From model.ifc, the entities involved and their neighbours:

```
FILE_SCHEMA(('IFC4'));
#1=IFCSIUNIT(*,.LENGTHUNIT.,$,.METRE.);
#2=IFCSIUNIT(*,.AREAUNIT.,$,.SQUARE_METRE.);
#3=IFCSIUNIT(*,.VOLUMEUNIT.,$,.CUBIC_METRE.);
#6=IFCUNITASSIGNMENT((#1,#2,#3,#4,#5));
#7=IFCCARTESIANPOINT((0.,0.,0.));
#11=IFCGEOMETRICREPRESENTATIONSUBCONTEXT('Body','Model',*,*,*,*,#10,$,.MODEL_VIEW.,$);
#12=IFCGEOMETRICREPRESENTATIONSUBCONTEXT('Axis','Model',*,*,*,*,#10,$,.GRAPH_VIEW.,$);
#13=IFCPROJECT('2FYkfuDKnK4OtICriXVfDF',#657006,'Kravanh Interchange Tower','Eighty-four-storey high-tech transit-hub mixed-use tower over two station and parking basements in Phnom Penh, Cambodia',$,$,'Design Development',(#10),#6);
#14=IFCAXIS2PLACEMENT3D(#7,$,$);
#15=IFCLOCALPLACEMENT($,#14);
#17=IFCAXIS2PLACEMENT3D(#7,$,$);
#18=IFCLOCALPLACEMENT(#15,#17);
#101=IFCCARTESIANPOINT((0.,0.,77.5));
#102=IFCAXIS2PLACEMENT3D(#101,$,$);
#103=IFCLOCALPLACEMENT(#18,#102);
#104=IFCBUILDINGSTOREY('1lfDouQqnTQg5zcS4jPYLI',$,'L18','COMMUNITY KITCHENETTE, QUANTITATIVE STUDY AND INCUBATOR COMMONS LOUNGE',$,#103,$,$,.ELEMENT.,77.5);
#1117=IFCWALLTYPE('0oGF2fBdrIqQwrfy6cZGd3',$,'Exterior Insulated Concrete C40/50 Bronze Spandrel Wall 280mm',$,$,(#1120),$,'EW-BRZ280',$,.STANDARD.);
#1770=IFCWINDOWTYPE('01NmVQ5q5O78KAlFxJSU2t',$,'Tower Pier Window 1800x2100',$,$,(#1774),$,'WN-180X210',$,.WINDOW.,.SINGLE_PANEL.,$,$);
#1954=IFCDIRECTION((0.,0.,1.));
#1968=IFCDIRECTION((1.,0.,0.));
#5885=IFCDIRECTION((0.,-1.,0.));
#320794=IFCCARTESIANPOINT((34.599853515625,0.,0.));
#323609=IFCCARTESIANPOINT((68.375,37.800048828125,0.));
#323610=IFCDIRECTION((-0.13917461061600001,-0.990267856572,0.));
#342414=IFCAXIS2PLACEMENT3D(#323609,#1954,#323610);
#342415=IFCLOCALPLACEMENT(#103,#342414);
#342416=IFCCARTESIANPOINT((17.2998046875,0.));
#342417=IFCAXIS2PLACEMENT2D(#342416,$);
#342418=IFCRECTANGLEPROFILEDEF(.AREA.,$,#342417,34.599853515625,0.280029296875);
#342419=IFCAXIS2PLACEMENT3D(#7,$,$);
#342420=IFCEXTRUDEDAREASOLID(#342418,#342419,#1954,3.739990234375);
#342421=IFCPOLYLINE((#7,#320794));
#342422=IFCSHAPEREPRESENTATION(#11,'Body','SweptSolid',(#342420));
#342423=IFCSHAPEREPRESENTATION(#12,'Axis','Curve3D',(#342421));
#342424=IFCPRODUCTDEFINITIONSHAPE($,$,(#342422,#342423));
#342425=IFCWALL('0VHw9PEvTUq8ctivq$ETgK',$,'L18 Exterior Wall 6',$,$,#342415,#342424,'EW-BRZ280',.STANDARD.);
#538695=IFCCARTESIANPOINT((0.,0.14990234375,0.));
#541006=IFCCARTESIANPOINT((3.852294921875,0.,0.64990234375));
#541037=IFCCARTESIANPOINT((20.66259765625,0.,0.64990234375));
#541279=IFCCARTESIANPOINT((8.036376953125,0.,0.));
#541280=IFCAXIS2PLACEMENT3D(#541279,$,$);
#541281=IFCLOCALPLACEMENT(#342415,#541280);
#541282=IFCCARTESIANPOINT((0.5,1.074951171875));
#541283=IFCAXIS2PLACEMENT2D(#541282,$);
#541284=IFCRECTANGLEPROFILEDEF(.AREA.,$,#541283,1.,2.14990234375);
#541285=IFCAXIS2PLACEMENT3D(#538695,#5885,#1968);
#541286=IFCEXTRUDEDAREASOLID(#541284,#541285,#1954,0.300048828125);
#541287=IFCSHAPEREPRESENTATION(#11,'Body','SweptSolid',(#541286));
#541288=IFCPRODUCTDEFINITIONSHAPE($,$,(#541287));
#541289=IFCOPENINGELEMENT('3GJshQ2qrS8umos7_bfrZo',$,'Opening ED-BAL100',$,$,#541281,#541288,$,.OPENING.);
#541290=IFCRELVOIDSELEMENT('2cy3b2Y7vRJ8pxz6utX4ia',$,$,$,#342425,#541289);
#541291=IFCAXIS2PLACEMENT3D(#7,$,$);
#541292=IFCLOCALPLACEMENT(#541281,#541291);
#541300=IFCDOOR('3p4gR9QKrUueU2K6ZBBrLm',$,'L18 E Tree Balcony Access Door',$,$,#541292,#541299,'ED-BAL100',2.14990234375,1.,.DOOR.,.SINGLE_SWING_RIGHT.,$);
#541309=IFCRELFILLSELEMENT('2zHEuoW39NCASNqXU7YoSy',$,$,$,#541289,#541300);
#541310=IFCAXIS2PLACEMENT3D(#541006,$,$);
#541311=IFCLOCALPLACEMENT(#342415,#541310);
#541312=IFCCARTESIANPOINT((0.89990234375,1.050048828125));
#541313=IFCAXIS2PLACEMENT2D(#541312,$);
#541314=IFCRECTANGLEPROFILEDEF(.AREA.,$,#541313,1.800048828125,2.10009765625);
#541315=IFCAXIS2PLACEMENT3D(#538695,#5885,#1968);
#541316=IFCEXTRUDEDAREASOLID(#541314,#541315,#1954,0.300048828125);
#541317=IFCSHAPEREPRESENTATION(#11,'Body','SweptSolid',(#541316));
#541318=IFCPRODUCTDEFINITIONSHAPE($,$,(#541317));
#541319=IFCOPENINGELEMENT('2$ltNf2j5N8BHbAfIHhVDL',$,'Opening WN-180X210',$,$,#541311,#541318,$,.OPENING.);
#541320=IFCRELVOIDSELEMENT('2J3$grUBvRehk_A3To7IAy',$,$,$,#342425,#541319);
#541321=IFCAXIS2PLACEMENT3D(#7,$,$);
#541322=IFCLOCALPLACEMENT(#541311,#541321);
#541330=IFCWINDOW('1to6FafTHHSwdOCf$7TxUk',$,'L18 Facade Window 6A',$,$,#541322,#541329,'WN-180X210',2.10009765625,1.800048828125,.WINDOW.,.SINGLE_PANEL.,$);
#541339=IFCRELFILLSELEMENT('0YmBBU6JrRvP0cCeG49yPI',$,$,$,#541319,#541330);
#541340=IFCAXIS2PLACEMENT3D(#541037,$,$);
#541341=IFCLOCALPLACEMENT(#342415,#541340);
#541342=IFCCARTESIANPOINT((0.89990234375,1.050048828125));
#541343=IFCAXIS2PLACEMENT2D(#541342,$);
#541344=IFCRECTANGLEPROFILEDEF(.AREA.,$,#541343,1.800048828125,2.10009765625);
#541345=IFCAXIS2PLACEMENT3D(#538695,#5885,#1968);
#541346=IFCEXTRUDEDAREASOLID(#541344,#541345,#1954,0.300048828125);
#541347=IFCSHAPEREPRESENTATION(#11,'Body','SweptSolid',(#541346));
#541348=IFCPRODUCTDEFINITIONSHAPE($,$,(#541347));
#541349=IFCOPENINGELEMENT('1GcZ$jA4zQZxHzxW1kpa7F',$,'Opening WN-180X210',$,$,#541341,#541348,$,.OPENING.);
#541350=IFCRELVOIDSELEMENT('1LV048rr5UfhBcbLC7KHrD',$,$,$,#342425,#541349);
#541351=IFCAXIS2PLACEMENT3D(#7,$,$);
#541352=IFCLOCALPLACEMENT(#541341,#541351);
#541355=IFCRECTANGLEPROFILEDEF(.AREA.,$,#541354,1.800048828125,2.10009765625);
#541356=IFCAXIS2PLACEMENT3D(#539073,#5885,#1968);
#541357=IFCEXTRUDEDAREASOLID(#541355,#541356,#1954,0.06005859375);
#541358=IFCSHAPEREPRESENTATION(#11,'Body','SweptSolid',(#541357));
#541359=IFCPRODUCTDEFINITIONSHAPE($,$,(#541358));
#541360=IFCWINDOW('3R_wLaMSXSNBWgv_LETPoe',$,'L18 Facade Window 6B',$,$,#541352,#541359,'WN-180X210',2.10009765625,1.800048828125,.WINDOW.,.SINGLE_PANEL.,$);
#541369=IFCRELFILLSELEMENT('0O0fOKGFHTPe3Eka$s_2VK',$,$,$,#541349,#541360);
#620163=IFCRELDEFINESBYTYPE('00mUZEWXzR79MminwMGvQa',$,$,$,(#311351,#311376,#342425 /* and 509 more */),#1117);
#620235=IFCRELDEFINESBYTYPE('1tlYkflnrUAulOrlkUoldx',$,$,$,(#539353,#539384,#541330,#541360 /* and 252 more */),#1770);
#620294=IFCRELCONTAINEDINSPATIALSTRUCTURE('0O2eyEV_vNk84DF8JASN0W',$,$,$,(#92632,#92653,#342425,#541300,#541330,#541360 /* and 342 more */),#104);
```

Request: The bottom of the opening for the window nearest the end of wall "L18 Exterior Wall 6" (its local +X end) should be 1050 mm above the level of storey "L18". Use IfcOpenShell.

```python
import numpy as np
import ifcopenshell
import ifcopenshell.api.geometry
import ifcopenshell.geom
import ifcopenshell.util.element
import ifcopenshell.util.placement
import ifcopenshell.util.shape
import ifcopenshell.util.unit

model = ifcopenshell.open("model.ifc")
unit_scale = ifcopenshell.util.unit.calculate_unit_scale(model)

window = model.by_guid("3R_wLaMSXSNBWgv_LETPoe")
opening = window.FillsVoids[0].RelatingOpeningElement
storey = ifcopenshell.util.element.get_container(window, ifc_class="IfcBuildingStorey")
level = ifcopenshell.util.placement.get_local_placement(storey.ObjectPlacement)[2, 3]

# The opening's origin need not be at the sill, so measure its lowest point.
shape = ifcopenshell.geom.create_shape(ifcopenshell.geom.settings(), opening)
bottom = ifcopenshell.util.shape.get_shape_bottom_elevation(shape, shape.geometry) / unit_scale
dz = level + 1.05 / unit_scale - bottom

shift = np.array([0.0, 0.0, dz])
# The window is placed relative to its opening, so it follows when the opening moves.
matrix = ifcopenshell.util.placement.get_local_placement(opening.ObjectPlacement)
matrix[:3, 3] += shift
ifcopenshell.api.geometry.edit_object_placement(
    model, product=opening, matrix=matrix, is_si=False, should_transform_children=True
)

print(f"moved by {dz * unit_scale:+.3f} m")

model.write("model_edited.ifc")
```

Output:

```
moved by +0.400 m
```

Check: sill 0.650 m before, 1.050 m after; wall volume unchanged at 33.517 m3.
